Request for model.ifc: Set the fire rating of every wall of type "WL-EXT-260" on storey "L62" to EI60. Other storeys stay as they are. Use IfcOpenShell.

First a look at what the model holds.

```python
import ifcopenshell
import ifcopenshell.util.element

model = ifcopenshell.open("model.ifc")
print(model.schema)
storey = next(s for s in model.by_type("IfcBuildingStorey") if s.Name == "L62")
walls = [e for e in ifcopenshell.util.element.get_decomposition(storey) if e.is_a("IfcWall")]
seen = {}
for e in walls:
    element_type = ifcopenshell.util.element.get_type(e)
    key = (element_type.Name if element_type != e and element_type else None, ifcopenshell.util.element.get_pset(e, "Pset_WallCommon", "FireRating"))
    seen[key] = seen.get(key, 0) + 1
for (name, value), count in sorted(seen.items(), key=str):
    print(count, "x", name, "|", value)
```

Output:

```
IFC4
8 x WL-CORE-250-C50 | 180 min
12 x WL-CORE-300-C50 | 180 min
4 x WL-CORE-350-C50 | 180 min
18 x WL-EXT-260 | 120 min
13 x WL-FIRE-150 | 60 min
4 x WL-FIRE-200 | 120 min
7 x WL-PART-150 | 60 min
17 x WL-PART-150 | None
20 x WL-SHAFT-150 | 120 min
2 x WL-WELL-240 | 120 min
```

```python
import ifcopenshell
import ifcopenshell.api.pset
import ifcopenshell.util.element

model = ifcopenshell.open("model.ifc")

storey = next(s for s in model.by_type("IfcBuildingStorey") if s.Name == "L62")
walls = [e for e in ifcopenshell.util.element.get_decomposition(storey) if e.is_a("IfcWall")]

count = 0
for e in walls:
    element_type = ifcopenshell.util.element.get_type(e)
    if element_type in (None, e) or element_type.Name != "WL-EXT-260":
        continue
    found = ifcopenshell.util.element.get_pset(e, "Pset_WallCommon", should_inherit=False)
    if found:
        pset = model.by_id(found["id"])
        if len(ifcopenshell.util.element.get_elements_by_pset(pset)) > 1:
            pset = ifcopenshell.api.pset.unshare_pset(model, products=[e], pset=pset)[0]
    else:
        pset = ifcopenshell.api.pset.add_pset(model, product=e, name="Pset_WallCommon")
    ifcopenshell.api.pset.edit_pset(model, pset=pset, properties={"FireRating": "EI60"})
    count += 1

print(count, "walls updated")

model.write("model_v2.ifc")
```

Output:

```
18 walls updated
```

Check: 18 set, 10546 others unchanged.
